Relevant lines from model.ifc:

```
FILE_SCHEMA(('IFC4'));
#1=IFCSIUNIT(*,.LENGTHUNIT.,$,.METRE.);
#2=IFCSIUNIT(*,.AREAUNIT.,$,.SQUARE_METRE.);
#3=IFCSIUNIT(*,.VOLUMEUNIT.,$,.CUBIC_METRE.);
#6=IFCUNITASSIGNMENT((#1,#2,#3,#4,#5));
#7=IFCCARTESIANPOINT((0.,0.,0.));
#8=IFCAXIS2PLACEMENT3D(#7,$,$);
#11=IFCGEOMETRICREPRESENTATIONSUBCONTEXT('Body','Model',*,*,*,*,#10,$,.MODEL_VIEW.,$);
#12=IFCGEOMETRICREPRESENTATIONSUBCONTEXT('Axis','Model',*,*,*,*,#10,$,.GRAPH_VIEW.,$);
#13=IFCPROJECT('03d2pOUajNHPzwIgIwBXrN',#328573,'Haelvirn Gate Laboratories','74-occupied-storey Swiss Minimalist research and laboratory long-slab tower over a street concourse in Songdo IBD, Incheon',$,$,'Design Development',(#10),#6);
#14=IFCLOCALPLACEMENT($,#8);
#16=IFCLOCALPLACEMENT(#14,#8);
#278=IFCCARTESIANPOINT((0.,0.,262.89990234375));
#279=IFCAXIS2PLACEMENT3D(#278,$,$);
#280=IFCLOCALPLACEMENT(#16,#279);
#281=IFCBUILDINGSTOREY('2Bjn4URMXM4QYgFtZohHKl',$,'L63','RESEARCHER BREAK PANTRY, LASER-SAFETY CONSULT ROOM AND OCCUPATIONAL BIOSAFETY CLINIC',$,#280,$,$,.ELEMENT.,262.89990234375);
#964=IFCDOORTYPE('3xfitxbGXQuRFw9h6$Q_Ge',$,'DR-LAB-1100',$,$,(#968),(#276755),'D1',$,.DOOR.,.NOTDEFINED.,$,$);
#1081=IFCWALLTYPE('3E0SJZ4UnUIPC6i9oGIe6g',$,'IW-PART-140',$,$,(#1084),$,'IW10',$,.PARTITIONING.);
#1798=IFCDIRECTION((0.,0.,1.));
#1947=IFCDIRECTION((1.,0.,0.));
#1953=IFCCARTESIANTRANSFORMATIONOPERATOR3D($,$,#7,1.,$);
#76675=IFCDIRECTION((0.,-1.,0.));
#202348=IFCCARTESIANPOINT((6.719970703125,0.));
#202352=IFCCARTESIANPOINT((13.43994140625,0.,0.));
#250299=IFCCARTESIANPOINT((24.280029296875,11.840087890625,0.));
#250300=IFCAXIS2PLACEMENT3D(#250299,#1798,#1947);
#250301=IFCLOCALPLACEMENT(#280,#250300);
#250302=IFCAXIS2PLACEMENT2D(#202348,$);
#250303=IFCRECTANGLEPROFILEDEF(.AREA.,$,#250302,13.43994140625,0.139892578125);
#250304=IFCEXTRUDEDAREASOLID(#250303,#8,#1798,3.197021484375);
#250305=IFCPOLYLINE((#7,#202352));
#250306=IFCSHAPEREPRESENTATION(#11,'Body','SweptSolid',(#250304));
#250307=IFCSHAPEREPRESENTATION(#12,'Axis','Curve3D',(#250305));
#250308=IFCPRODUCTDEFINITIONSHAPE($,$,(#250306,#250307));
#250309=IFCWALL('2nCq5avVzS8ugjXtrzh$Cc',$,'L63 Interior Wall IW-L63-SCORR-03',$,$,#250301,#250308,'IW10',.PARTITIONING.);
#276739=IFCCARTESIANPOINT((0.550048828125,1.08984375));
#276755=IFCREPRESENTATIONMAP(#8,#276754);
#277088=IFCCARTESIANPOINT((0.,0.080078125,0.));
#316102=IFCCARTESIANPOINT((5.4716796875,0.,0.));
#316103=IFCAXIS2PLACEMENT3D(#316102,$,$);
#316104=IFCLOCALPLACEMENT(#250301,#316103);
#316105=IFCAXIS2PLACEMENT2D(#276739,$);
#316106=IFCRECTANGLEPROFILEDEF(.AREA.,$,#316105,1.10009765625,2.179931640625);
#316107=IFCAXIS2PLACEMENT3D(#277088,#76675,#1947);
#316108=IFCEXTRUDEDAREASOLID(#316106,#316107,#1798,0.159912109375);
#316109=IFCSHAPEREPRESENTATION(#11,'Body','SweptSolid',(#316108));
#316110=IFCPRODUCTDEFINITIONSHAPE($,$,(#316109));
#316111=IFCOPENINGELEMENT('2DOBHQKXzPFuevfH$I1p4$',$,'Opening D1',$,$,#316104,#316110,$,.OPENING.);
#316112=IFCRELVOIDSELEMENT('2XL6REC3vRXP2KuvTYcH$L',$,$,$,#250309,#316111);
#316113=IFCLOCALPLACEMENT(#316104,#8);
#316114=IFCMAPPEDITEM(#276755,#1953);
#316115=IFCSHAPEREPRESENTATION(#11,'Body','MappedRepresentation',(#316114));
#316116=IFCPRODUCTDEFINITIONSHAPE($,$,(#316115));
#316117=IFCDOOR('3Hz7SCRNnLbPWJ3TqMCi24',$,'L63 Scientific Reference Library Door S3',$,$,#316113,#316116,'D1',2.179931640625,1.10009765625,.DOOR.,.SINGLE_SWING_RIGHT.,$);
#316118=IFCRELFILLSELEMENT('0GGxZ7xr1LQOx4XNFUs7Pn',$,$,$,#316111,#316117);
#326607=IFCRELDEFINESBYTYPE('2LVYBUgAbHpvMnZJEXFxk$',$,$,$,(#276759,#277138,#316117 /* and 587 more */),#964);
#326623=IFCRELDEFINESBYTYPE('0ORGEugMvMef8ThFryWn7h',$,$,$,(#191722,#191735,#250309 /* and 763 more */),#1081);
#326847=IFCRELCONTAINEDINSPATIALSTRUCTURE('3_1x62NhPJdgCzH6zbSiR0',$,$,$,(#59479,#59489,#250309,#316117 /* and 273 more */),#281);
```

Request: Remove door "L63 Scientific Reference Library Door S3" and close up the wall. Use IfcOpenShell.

```python
import ifcopenshell
import ifcopenshell.api.feature
import ifcopenshell.api.root
import ifcopenshell.geom
import ifcopenshell.util.shape

model = ifcopenshell.open("model.ifc")
settings = ifcopenshell.geom.settings()


def volume(element):
    """Net volume in cubic metres, openings subtracted."""
    shape = ifcopenshell.geom.create_shape(settings, element)
    return ifcopenshell.util.shape.get_volume(shape.geometry)


door = model.by_guid("3Hz7SCRNnLbPWJ3TqMCi24")
opening = door.FillsVoids[0].RelatingOpeningElement
wall = opening.VoidsElements[0].RelatingBuildingElement
before = volume(wall)

ifcopenshell.api.root.remove_product(model, product=door)
ifcopenshell.api.feature.remove_feature(model, feature=opening)

after = volume(wall)

print(f"wall volume {before:.3f} -> {after:.3f} m3")

model.write("model_updated.ifc")
```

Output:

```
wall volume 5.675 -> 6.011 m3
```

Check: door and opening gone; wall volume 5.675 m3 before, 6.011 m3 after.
